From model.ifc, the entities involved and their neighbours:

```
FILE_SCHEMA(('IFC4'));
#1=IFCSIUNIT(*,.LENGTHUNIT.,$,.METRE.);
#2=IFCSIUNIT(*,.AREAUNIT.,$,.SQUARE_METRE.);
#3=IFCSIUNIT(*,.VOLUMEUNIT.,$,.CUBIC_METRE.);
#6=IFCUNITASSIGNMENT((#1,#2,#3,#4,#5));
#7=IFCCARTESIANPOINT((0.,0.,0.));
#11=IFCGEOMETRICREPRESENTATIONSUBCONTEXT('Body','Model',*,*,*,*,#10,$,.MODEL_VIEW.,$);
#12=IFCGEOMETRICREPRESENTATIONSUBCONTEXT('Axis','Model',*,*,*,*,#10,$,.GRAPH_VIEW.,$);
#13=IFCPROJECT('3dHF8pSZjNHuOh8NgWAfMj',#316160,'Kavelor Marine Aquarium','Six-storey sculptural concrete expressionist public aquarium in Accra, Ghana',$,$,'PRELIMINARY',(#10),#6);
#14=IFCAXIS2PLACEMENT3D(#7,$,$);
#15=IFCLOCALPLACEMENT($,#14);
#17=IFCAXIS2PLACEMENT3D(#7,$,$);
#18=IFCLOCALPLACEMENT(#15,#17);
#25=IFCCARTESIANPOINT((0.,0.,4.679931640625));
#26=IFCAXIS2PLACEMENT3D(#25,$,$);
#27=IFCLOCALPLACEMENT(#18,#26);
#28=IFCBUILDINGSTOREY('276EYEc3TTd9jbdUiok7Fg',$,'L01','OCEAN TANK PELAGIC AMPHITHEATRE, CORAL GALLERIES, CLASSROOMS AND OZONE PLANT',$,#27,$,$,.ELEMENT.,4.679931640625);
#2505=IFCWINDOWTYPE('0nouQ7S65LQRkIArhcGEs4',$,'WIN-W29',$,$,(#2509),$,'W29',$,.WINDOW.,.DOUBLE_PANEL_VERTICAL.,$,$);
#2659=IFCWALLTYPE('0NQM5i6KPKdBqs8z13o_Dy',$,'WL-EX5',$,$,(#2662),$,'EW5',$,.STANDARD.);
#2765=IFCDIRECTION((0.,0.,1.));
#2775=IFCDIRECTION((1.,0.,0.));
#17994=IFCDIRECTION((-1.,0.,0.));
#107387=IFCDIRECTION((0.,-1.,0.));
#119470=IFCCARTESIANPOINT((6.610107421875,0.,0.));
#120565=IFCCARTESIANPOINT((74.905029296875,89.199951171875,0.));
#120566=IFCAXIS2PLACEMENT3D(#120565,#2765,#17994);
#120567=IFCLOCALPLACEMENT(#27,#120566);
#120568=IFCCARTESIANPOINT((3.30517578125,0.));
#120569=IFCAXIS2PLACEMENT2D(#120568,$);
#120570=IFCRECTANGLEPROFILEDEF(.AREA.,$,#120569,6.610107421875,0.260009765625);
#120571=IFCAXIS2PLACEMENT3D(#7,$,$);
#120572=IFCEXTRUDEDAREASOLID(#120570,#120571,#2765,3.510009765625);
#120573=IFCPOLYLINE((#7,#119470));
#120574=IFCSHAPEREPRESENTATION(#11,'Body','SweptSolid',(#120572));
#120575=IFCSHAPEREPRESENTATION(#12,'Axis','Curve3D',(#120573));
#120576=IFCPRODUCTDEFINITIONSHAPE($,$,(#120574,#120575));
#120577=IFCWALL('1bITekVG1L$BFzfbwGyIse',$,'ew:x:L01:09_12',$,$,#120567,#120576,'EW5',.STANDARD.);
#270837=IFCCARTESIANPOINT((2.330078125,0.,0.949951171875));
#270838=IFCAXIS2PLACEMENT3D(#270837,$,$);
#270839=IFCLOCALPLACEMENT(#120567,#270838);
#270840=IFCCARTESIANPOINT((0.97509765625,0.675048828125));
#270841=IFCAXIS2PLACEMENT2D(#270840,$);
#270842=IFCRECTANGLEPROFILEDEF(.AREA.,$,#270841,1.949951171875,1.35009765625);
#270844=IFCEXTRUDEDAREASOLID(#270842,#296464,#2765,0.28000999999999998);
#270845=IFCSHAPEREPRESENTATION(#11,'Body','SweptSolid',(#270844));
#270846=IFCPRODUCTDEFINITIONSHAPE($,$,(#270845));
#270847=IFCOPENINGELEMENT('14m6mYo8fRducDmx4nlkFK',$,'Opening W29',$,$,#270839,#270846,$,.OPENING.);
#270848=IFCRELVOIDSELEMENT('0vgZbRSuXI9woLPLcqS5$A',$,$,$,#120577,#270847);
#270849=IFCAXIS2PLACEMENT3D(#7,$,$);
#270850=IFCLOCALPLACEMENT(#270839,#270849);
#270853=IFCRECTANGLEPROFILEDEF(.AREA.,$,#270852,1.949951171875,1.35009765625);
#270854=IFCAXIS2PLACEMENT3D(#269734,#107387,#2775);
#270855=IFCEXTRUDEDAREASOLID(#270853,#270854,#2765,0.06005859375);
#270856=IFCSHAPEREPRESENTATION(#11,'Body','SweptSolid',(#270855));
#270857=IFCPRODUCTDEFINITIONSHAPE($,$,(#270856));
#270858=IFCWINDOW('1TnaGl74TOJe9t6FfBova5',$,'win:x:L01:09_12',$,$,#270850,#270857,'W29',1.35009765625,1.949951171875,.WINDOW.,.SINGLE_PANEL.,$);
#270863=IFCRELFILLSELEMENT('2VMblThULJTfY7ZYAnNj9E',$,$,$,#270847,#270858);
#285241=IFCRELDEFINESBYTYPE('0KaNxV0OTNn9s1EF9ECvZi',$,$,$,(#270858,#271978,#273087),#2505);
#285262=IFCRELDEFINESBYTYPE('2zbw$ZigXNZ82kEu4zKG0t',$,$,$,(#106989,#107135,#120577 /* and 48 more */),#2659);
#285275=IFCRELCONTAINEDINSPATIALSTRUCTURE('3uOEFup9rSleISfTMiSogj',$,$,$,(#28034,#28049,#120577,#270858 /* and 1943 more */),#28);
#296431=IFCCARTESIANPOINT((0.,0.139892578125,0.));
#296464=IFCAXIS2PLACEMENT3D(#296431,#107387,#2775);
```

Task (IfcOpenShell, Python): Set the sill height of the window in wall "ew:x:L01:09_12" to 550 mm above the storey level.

```python
import numpy as np
import ifcopenshell
import ifcopenshell.api.geometry
import ifcopenshell.geom
import ifcopenshell.util.element
import ifcopenshell.util.placement
import ifcopenshell.util.shape
import ifcopenshell.util.unit

model = ifcopenshell.open("model.ifc")
unit_scale = ifcopenshell.util.unit.calculate_unit_scale(model)

window = model.by_guid("1TnaGl74TOJe9t6FfBova5")
opening = window.FillsVoids[0].RelatingOpeningElement
storey = ifcopenshell.util.element.get_container(window, ifc_class="IfcBuildingStorey")
level = ifcopenshell.util.placement.get_local_placement(storey.ObjectPlacement)[2, 3]

# The opening's origin need not be at the sill, so measure its lowest point.
shape = ifcopenshell.geom.create_shape(ifcopenshell.geom.settings(), opening)
bottom = ifcopenshell.util.shape.get_shape_bottom_elevation(shape, shape.geometry) / unit_scale
dz = level + 0.55 - bottom

shift = np.array([0.0, 0.0, dz])
# The window is placed relative to its opening, so it follows when the opening moves.
matrix = ifcopenshell.util.placement.get_local_placement(opening.ObjectPlacement)
matrix[:3, 3] += shift
ifcopenshell.api.geometry.edit_object_placement(
    model, product=opening, matrix=matrix, is_si=False, should_transform_children=True
)

print(f"moved by {dz * unit_scale:+.3f} m")

model.write("model_v2.ifc")
```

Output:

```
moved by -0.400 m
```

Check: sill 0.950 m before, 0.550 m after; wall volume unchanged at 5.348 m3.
